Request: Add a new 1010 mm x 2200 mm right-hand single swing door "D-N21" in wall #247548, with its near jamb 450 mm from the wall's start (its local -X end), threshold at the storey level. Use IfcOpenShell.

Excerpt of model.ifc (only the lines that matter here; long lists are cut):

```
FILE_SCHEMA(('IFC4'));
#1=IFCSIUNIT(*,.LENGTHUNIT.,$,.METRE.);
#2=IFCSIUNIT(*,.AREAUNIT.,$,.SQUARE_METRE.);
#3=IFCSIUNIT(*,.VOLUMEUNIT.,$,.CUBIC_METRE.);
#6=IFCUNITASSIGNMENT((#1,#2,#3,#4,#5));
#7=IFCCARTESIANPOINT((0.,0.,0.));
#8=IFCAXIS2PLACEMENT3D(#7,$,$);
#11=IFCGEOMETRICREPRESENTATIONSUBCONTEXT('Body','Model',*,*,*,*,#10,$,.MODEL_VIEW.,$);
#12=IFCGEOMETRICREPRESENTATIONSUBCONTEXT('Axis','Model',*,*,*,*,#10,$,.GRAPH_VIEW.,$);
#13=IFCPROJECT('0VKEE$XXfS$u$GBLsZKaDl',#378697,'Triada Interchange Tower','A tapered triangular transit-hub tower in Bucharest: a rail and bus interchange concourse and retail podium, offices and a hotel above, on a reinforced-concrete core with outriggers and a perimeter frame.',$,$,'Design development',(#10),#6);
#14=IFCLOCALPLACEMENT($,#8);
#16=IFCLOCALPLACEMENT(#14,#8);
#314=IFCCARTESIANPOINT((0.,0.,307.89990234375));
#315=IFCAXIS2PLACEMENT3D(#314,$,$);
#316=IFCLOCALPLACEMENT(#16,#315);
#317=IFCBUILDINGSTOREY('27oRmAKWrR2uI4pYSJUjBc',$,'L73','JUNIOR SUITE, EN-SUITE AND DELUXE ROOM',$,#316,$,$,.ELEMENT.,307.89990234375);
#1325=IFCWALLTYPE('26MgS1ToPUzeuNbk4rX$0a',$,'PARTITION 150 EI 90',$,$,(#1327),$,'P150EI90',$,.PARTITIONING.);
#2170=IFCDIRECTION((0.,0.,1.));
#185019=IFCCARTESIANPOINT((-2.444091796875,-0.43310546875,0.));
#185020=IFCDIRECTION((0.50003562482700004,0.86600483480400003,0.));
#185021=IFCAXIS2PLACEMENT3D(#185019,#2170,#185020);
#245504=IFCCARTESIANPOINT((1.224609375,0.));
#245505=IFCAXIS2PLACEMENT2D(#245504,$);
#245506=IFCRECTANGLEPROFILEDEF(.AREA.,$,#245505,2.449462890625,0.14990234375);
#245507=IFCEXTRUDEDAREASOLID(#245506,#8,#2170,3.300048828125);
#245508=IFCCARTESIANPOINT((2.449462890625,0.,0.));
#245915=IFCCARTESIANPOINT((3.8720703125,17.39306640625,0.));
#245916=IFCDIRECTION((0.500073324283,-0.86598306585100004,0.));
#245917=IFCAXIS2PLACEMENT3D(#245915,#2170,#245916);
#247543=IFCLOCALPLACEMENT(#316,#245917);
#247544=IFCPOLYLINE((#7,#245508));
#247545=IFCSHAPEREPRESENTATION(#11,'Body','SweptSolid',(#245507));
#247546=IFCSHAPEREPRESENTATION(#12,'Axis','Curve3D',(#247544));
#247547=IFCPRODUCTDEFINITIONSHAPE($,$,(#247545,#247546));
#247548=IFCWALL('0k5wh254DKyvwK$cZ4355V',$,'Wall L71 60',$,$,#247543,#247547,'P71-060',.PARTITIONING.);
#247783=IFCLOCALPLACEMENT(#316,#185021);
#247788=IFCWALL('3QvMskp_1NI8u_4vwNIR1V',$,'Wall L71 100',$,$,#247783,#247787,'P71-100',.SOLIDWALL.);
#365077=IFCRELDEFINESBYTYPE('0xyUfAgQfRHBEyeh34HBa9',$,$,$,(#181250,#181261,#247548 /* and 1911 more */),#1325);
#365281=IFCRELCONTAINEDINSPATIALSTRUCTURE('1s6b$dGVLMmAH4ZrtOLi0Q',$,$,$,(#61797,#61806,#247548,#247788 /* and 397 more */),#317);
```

```python
import numpy as np
import ifcopenshell
import ifcopenshell.api.feature
import ifcopenshell.api.geometry
import ifcopenshell.api.root
import ifcopenshell.api.spatial
import ifcopenshell.geom
import ifcopenshell.util.element
import ifcopenshell.util.placement
import ifcopenshell.util.representation
import ifcopenshell.util.shape
import ifcopenshell.util.unit

model = ifcopenshell.open("model.ifc")
unit_scale = ifcopenshell.util.unit.calculate_unit_scale(model)
settings = ifcopenshell.geom.settings()


def volume(element):
    """Net volume in cubic metres, openings subtracted."""
    shape = ifcopenshell.geom.create_shape(settings, element)
    return ifcopenshell.util.shape.get_volume(shape.geometry)


wall = model.by_guid("0k5wh254DKyvwK$cZ4355V")
storey = ifcopenshell.util.element.get_container(wall, ifc_class="IfcBuildingStorey")
context = ifcopenshell.util.representation.get_context(model, "Model", "Body", "MODEL_VIEW")
before = volume(wall)

width, height, from_end, sill = 1.01, 2.2, 0.45, 0.0  # metres

# The wall runs along its own X axis, and the end named is its -X end.
wall_shape = ifcopenshell.geom.create_shape(settings, wall)
x, y, z = ifcopenshell.util.shape.get_vertices(wall_shape.geometry).T
start = x.min() + from_end
face, thickness = float(y.min()), float(y.max() - y.min())
wall_matrix = ifcopenshell.util.placement.get_local_placement(wall.ObjectPlacement)
level = ifcopenshell.util.placement.get_local_placement(storey.ObjectPlacement)[2, 3]


def in_wall(x, y):
    """Placement at x, y metres in the wall's axes, at sill height."""
    matrix = wall_matrix.copy()
    matrix[:, 3] = wall_matrix @ np.array([x / unit_scale, y / unit_scale, 0.0, 1.0])
    matrix[2, 3] = level + sill / unit_scale
    return matrix


# Opening: a box that overshoots both wall faces by 50 mm.
opening = ifcopenshell.api.root.create_entity(model, ifc_class="IfcOpeningElement", predefined_type="OPENING")
box = ifcopenshell.api.geometry.add_wall_representation(
    model, context=context, length=width, height=height, thickness=thickness + 0.1
)
ifcopenshell.api.geometry.assign_representation(model, product=opening, representation=box)
ifcopenshell.api.geometry.edit_object_placement(model, product=opening, matrix=in_wall(start, face - 0.05), is_si=False)
ifcopenshell.api.feature.add_feature(model, feature=opening, element=wall)

door = ifcopenshell.api.root.create_entity(model, ifc_class="IfcDoor", name="D-N21", predefined_type="DOOR")
door.OverallWidth, door.OverallHeight = width / unit_scale, height / unit_scale
door.OperationType = "SINGLE_SWING_RIGHT"
body = ifcopenshell.api.geometry.add_door_representation(
    model,
    context=context,
    overall_width=door.OverallWidth,
    overall_height=door.OverallHeight,
    operation_type="SINGLE_SWING_RIGHT",
    lining_properties={"LiningDepth": thickness / unit_scale, "ThresholdDepth": thickness / unit_scale},
)
ifcopenshell.api.geometry.assign_representation(model, product=door, representation=body)
ifcopenshell.api.spatial.assign_container(model, products=[door], relating_structure=storey)
ifcopenshell.api.feature.add_filling(model, opening=opening, element=door)

# The lining spans the wall, so the door starts at the wall face.
ifcopenshell.api.geometry.edit_object_placement(model, product=door, matrix=in_wall(start, face), is_si=False)

after = volume(wall)

print(f"wall volume {before:.3f} -> {after:.3f} m3")

model.write("model_edited.ifc")
```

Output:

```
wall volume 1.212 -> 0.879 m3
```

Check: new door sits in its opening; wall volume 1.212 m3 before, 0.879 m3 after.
